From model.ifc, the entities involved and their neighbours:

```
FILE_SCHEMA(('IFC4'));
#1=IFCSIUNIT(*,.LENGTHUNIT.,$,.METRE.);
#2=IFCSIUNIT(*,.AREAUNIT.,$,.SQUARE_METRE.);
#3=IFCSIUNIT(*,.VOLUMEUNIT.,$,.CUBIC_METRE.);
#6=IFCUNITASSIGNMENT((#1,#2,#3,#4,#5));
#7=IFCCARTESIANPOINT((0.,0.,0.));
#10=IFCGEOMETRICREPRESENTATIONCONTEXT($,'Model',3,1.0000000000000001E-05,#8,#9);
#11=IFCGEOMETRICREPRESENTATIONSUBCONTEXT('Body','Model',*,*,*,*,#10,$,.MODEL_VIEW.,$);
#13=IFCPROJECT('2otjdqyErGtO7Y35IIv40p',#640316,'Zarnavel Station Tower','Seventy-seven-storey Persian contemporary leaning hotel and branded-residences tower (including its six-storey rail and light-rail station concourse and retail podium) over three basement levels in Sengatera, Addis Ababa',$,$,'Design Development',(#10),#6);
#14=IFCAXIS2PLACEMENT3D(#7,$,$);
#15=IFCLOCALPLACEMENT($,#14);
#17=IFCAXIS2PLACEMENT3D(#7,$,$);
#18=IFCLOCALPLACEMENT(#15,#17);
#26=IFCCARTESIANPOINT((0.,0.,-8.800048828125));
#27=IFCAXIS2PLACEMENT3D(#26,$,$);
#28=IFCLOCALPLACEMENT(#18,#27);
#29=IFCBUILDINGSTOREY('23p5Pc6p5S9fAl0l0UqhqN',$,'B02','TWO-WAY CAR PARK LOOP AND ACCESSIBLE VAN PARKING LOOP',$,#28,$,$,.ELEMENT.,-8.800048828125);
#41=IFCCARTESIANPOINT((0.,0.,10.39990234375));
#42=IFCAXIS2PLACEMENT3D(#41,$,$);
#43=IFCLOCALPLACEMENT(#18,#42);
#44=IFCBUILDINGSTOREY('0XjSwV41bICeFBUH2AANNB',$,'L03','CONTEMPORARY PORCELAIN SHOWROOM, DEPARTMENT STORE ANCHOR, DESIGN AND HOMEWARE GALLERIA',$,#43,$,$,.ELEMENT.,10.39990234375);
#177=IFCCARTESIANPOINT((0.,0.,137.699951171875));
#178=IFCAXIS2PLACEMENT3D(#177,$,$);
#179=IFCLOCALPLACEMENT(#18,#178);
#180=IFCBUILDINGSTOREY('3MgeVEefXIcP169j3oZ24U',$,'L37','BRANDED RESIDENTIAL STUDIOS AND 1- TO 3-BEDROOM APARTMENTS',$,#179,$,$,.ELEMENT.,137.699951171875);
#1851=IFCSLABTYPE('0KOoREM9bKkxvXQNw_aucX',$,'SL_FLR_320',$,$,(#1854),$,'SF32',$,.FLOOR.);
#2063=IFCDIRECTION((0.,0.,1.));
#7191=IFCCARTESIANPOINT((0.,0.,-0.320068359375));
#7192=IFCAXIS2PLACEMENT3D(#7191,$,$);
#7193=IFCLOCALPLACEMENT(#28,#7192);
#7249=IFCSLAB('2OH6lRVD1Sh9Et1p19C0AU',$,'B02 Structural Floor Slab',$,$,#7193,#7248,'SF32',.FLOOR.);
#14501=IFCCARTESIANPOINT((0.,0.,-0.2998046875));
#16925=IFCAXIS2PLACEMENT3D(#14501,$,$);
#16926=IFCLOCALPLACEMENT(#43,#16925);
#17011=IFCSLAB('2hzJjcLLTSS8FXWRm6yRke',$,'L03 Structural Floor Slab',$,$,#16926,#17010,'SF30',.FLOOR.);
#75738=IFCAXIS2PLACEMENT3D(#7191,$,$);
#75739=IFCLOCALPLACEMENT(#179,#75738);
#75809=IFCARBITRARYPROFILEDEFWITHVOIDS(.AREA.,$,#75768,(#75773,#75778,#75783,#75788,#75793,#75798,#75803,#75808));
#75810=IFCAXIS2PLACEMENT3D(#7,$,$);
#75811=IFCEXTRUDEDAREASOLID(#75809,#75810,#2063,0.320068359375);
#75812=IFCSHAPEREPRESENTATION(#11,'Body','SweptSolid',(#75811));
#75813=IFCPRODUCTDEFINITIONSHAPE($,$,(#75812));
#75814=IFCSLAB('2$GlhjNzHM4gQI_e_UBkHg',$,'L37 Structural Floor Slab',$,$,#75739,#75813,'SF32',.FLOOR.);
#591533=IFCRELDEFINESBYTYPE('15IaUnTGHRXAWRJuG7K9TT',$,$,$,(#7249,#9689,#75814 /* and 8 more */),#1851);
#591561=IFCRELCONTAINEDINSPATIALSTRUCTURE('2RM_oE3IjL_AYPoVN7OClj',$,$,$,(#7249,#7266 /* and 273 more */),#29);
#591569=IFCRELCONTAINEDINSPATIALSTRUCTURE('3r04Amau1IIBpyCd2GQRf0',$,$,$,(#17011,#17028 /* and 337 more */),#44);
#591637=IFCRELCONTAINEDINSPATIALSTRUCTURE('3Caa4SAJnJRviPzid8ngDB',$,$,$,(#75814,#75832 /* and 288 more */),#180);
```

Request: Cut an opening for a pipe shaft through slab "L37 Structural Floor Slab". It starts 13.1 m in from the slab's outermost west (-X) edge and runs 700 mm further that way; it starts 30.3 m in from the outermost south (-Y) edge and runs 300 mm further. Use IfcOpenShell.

```python
import numpy as np
import ifcopenshell
import ifcopenshell.api.feature
import ifcopenshell.api.geometry
import ifcopenshell.api.root
import ifcopenshell.geom
import ifcopenshell.util.placement
import ifcopenshell.util.representation
import ifcopenshell.util.shape
import ifcopenshell.util.unit

model = ifcopenshell.open("model.ifc")
unit_scale = ifcopenshell.util.unit.calculate_unit_scale(model)
settings = ifcopenshell.geom.settings()


def volume(element):
    """Net volume in cubic metres, openings subtracted."""
    shape = ifcopenshell.geom.create_shape(settings, element)
    return ifcopenshell.util.shape.get_volume(shape.geometry)


slab = model.by_guid("2$GlhjNzHM4gQI_e_UBkHg")
before = volume(slab)

# Extent in the slab's own axes, in metres. The edges named are its -X and -Y sides.
slab_shape = ifcopenshell.geom.create_shape(settings, slab)
vertices = ifcopenshell.util.shape.get_vertices(slab_shape.geometry)
x_min, y_min, bottom = vertices.min(axis=0)
top = vertices[:, 2].max()

opening = ifcopenshell.api.root.create_entity(model, ifc_class="IfcOpeningElement", name="Pipe shaft opening", predefined_type="OPENING")
context = ifcopenshell.util.representation.get_context(model, "Model", "Body", "MODEL_VIEW")
width, depth = 0.7, 0.3
outline = [(0.0, 0.0), (width, 0.0), (width, depth), (0.0, depth), (0.0, 0.0)]
# Overshoot both faces by 50 mm so the cut is clean.
shape = ifcopenshell.api.geometry.add_slab_representation(
    model, context=context, depth=top - bottom + 0.1, polyline=outline
)
ifcopenshell.api.geometry.assign_representation(model, product=opening, representation=shape)

matrix = ifcopenshell.util.placement.get_local_placement(slab.ObjectPlacement)
matrix[:, 3] = matrix @ np.append(np.array([x_min + 13.1, y_min + 30.3, bottom - 0.05]) / unit_scale, 1.0)
ifcopenshell.api.geometry.edit_object_placement(model, product=opening, matrix=matrix, is_si=False)
ifcopenshell.api.feature.add_feature(model, feature=opening, element=slab)

after = volume(slab)

print(f"slab volume {before:.3f} -> {after:.3f} m3")

model.write("model_rev.ifc")
```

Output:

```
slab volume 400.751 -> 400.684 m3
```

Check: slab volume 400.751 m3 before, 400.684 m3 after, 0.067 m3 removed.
